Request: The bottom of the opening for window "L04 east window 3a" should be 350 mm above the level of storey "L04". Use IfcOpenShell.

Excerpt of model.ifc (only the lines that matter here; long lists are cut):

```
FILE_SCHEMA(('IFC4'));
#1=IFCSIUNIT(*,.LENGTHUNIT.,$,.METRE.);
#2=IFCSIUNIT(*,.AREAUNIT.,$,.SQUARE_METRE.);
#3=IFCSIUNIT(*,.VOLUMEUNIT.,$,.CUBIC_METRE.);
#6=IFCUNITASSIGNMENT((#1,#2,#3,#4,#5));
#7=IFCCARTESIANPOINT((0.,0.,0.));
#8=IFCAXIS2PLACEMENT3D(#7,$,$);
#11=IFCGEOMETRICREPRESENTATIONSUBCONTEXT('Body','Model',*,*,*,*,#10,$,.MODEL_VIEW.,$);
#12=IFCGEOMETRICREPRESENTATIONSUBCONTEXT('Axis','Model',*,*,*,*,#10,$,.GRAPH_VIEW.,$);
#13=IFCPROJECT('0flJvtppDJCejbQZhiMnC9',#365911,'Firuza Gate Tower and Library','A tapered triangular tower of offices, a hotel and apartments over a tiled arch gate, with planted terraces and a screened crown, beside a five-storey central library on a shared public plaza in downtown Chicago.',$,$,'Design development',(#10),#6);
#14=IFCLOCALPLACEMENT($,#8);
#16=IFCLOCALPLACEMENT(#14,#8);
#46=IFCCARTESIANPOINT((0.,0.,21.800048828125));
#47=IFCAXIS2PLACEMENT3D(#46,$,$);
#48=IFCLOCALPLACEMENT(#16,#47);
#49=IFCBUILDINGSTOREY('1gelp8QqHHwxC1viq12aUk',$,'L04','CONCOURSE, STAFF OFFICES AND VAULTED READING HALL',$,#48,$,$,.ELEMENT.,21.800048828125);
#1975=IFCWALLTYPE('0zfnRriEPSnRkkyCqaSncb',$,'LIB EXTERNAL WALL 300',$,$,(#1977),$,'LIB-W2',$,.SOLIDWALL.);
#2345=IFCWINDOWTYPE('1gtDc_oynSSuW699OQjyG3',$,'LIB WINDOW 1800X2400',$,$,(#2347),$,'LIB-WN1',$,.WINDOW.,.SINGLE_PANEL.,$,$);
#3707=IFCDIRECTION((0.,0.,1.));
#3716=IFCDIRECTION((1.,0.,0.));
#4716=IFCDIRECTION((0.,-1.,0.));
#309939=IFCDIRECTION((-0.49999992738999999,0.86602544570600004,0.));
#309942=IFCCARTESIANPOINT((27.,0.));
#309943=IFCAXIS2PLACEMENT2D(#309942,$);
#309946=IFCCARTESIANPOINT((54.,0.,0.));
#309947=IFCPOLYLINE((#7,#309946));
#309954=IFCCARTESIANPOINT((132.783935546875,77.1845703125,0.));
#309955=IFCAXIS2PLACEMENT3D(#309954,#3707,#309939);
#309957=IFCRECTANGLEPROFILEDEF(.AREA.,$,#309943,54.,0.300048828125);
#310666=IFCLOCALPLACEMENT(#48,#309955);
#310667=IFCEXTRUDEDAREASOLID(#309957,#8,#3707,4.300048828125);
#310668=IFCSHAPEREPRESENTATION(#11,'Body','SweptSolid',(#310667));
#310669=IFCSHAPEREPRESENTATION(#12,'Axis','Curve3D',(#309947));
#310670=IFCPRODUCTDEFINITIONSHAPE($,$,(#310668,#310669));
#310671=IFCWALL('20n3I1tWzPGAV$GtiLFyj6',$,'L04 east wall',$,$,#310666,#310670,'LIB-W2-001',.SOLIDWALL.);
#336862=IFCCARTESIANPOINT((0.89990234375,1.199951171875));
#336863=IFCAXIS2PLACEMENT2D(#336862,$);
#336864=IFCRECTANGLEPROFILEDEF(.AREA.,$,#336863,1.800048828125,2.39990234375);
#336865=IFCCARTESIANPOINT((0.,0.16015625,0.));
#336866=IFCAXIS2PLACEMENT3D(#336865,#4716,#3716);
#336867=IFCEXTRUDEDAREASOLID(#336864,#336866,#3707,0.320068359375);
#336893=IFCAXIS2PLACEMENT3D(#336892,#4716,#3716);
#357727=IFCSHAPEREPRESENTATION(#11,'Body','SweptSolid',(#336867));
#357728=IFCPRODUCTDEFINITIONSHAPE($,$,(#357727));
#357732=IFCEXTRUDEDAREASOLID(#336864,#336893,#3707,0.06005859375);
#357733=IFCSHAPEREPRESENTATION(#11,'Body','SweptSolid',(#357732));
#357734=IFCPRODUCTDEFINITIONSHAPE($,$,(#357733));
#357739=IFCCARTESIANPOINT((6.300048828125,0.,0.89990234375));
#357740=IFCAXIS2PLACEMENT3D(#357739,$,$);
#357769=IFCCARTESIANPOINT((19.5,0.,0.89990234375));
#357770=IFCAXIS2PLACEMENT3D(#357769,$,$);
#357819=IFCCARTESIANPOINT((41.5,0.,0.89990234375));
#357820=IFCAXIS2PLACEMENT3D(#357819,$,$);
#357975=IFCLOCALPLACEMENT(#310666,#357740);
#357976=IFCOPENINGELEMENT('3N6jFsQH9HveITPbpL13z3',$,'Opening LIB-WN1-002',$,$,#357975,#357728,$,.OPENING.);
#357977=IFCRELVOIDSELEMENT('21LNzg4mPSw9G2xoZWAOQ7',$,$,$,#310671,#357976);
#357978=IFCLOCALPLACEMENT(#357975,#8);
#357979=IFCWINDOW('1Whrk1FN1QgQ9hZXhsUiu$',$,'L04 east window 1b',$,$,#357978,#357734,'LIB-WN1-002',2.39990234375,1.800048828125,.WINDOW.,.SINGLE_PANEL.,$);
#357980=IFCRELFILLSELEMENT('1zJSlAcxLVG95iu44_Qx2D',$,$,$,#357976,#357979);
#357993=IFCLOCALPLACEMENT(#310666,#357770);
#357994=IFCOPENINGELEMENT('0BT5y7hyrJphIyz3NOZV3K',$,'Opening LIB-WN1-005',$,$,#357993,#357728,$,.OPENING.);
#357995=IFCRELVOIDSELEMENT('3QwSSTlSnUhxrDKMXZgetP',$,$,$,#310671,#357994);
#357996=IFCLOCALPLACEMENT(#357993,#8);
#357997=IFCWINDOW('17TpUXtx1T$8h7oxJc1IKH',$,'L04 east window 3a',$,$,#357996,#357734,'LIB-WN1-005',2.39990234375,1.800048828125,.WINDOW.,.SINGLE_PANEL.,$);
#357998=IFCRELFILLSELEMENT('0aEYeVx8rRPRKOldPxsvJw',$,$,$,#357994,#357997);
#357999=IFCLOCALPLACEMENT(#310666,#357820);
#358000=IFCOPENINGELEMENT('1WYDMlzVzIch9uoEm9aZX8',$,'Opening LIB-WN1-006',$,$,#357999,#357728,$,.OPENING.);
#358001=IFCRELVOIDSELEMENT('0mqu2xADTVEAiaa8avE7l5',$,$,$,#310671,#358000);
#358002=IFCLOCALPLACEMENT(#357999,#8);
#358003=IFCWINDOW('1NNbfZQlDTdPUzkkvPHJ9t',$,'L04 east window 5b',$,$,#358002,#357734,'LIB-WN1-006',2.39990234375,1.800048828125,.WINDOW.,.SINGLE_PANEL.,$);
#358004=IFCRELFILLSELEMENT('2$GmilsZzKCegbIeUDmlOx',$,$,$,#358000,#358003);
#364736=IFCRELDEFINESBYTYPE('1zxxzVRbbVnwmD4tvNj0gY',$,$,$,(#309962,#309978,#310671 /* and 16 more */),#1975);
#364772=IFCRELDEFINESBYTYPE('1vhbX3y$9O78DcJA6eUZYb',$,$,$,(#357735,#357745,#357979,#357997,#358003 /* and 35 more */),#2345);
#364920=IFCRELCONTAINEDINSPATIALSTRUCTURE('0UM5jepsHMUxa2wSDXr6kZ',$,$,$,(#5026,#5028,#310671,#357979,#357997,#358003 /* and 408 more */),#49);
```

```python
import numpy as np
import ifcopenshell
import ifcopenshell.api.geometry
import ifcopenshell.geom
import ifcopenshell.util.element
import ifcopenshell.util.placement
import ifcopenshell.util.shape
import ifcopenshell.util.unit

model = ifcopenshell.open("model.ifc")
unit_scale = ifcopenshell.util.unit.calculate_unit_scale(model)

window = model.by_guid("17TpUXtx1T$8h7oxJc1IKH")
opening = window.FillsVoids[0].RelatingOpeningElement
storey = ifcopenshell.util.element.get_container(window, ifc_class="IfcBuildingStorey")
level = ifcopenshell.util.placement.get_local_placement(storey.ObjectPlacement)[2, 3]

# The opening's origin need not be at the sill, so measure its lowest point.
shape = ifcopenshell.geom.create_shape(ifcopenshell.geom.settings(), opening)
bottom = ifcopenshell.util.shape.get_shape_bottom_elevation(shape, shape.geometry) / unit_scale
dz = level + 0.35 / unit_scale - bottom

shift = np.array([0.0, 0.0, dz])
# The window is placed relative to its opening, so it follows when the opening moves.
matrix = ifcopenshell.util.placement.get_local_placement(opening.ObjectPlacement)
matrix[:3, 3] += shift
ifcopenshell.api.geometry.edit_object_placement(
    model, product=opening, matrix=matrix, is_si=False, should_transform_children=True
)

print(f"moved by {dz * unit_scale:+.3f} m")

model.write("model_rev.ifc")
```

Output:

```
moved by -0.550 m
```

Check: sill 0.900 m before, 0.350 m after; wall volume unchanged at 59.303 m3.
